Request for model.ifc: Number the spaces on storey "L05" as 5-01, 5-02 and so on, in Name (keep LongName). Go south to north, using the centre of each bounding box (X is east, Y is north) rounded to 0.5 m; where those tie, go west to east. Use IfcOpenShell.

First a look at what the model holds.

```python
import ifcopenshell
import ifcopenshell.util.element
import ifcopenshell.util.placement

model = ifcopenshell.open("model.ifc")
print(model.schema)
storey = next(s for s in model.by_type("IfcBuildingStorey") if s.Name == "L05")
spaces = [e for e in ifcopenshell.util.element.get_decomposition(storey) if e.is_a("IfcSpace")]
for e in sorted(spaces, key=lambda e: e.id()):
    origin = ifcopenshell.util.placement.get_local_placement(e.ObjectPlacement)[:3, 3]
    print(e.id(), e.Name, e.LongName, origin.round(2) + 0.0, sep=" | ")
```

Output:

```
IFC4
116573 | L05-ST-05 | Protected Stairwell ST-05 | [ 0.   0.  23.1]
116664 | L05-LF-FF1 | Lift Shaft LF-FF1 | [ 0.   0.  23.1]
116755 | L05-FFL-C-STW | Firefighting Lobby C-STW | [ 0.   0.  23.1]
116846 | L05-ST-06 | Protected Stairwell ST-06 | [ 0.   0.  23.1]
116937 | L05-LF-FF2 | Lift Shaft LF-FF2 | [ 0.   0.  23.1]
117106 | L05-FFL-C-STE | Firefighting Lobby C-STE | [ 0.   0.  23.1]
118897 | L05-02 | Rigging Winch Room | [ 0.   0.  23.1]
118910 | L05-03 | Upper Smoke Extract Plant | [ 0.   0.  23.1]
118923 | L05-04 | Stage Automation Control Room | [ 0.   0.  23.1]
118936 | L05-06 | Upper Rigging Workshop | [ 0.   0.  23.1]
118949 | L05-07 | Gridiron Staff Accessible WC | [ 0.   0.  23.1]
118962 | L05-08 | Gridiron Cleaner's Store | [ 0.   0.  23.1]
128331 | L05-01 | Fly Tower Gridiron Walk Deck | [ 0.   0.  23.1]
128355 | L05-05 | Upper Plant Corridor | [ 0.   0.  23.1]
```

```python
import ifcopenshell
import ifcopenshell.geom
import ifcopenshell.util.element
import ifcopenshell.util.shape

model = ifcopenshell.open("model.ifc")
settings = ifcopenshell.geom.settings()
settings.set("use-world-coords", True)


def centre(element):
    shape = ifcopenshell.geom.create_shape(settings, element)
    return ifcopenshell.util.shape.get_bbox_centroid(shape.geometry)


storey = next(s for s in model.by_type("IfcBuildingStorey") if s.Name == "L05")
spaces = [e for e in ifcopenshell.util.element.get_decomposition(storey) if e.is_a("IfcSpace")]

# Insertion points can sit at a corner or the storey origin, so sort by the geometry (in metres).
centres = {e: centre(e) for e in spaces}
spaces.sort(key=lambda e: (round(centres[e][1] / 0.5), centres[e][0]))

for i, e in enumerate(spaces, start=1):
    number = f"5-{i:02d}"
    e.Name = number
    print(e.id(), number)

model.write("model_v2.ifc")
```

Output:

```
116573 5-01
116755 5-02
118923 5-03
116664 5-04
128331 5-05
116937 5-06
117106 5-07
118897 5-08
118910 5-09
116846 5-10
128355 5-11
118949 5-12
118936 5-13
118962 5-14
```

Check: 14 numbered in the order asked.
